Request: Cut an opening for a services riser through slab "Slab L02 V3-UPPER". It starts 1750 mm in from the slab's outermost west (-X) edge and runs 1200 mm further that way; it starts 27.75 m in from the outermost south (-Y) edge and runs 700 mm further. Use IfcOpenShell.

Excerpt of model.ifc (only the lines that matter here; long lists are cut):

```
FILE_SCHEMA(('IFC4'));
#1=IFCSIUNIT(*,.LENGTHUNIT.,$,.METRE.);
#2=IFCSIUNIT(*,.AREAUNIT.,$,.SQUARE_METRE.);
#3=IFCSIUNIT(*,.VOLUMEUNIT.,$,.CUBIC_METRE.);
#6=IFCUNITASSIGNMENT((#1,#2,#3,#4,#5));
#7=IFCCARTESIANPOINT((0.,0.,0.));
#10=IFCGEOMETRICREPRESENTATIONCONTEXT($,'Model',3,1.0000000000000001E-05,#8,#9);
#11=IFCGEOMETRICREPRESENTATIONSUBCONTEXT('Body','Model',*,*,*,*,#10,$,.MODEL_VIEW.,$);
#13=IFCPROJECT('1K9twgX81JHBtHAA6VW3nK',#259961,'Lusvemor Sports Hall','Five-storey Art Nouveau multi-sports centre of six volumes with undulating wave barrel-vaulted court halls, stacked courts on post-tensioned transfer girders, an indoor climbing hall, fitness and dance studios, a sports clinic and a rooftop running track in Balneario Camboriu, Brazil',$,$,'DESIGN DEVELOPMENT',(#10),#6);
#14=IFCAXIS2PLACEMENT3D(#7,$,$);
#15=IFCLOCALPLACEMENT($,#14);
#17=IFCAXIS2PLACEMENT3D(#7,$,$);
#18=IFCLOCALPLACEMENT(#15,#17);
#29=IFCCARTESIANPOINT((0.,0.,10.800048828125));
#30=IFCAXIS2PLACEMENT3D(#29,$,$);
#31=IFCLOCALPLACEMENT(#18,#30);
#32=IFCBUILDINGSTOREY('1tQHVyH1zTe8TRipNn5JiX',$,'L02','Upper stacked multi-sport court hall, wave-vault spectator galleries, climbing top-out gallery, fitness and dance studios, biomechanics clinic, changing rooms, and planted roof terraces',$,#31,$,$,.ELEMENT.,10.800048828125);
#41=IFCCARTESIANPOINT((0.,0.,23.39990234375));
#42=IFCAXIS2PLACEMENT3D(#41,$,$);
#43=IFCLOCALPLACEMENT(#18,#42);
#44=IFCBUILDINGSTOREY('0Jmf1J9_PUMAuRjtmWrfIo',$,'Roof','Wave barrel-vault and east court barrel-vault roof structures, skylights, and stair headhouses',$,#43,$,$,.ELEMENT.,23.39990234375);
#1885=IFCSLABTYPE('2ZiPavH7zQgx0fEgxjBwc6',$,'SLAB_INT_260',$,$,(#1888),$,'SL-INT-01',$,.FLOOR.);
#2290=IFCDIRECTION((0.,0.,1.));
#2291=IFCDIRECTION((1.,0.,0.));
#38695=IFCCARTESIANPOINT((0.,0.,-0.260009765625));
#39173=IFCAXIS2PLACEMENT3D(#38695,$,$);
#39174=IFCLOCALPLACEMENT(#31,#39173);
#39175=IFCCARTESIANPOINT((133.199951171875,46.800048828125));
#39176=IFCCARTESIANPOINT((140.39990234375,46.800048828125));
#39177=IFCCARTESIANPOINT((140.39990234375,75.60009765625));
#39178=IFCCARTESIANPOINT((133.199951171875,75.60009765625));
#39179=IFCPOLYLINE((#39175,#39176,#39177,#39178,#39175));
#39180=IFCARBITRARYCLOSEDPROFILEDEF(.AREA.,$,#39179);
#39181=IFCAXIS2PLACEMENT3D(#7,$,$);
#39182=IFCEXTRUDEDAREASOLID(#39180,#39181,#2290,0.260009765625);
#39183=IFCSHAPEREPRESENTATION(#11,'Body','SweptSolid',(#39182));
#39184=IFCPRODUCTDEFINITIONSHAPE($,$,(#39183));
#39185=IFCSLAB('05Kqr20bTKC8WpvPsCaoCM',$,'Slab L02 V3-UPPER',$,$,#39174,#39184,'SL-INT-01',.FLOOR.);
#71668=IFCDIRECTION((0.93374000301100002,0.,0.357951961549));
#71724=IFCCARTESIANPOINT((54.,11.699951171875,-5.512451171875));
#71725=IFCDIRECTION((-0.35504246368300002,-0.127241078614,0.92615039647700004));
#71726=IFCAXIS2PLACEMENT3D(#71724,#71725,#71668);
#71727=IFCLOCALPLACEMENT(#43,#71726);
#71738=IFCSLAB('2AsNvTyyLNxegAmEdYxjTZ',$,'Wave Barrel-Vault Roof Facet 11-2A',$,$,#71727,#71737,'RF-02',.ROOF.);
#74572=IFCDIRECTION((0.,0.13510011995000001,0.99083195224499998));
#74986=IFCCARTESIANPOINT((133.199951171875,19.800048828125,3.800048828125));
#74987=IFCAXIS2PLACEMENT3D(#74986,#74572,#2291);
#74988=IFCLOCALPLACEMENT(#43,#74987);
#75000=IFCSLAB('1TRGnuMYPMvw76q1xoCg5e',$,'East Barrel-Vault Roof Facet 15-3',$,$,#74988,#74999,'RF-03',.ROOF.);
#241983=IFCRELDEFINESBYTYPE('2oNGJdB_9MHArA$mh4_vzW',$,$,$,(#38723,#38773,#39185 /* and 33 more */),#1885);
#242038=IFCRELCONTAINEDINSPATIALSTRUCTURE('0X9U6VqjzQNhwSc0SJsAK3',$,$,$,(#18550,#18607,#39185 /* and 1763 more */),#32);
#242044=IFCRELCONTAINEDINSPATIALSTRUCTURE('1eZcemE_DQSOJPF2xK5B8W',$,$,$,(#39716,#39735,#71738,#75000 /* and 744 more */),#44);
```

```python
import numpy as np
import ifcopenshell
import ifcopenshell.api.feature
import ifcopenshell.api.geometry
import ifcopenshell.api.root
import ifcopenshell.geom
import ifcopenshell.util.placement
import ifcopenshell.util.representation
import ifcopenshell.util.shape
import ifcopenshell.util.unit

model = ifcopenshell.open("model.ifc")
unit_scale = ifcopenshell.util.unit.calculate_unit_scale(model)
settings = ifcopenshell.geom.settings()


def volume(element):
    """Net volume in cubic metres, openings subtracted."""
    shape = ifcopenshell.geom.create_shape(settings, element)
    return ifcopenshell.util.shape.get_volume(shape.geometry)


slab = model.by_guid("05Kqr20bTKC8WpvPsCaoCM")
before = volume(slab)

# Extent in the slab's own axes, in metres. The edges named are its -X and -Y sides.
slab_shape = ifcopenshell.geom.create_shape(settings, slab)
vertices = ifcopenshell.util.shape.get_vertices(slab_shape.geometry)
x_min, y_min, bottom = vertices.min(axis=0)
top = vertices[:, 2].max()

opening = ifcopenshell.api.root.create_entity(model, ifc_class="IfcOpeningElement", name="Services riser opening", predefined_type="OPENING")
context = ifcopenshell.util.representation.get_context(model, "Model", "Body", "MODEL_VIEW")
width, depth = 1.2, 0.7
outline = [(0.0, 0.0), (width, 0.0), (width, depth), (0.0, depth), (0.0, 0.0)]
# Overshoot both faces by 50 mm so the cut is clean.
shape = ifcopenshell.api.geometry.add_slab_representation(
    model, context=context, depth=top - bottom + 0.1, polyline=outline
)
ifcopenshell.api.geometry.assign_representation(model, product=opening, representation=shape)

matrix = ifcopenshell.util.placement.get_local_placement(slab.ObjectPlacement)
matrix[:, 3] = matrix @ np.append(np.array([x_min + 1.75, y_min + 27.75, bottom - 0.05]) / unit_scale, 1.0)
ifcopenshell.api.geometry.edit_object_placement(model, product=opening, matrix=matrix, is_si=False)
ifcopenshell.api.feature.add_feature(model, feature=opening, element=slab)

after = volume(slab)

print(f"slab volume {before:.3f} -> {after:.3f} m3")

model.write("model-out.ifc")
```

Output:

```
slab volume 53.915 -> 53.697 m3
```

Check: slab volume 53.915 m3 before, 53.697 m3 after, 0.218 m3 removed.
